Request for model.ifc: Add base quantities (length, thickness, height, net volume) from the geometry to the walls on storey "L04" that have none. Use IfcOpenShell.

First a look at what the model holds.

```python
import ifcopenshell
import ifcopenshell.util.element
import ifcopenshell.util.unit

model = ifcopenshell.open("model.ifc")
print(model.schema)
for unit_type in ("LENGTHUNIT", "AREAUNIT", "VOLUMEUNIT"):
    print(unit_type, ifcopenshell.util.unit.calculate_unit_scale(model, unit_type))
storey = next(s for s in model.by_type("IfcBuildingStorey") if s.Name == "L04")
walls = [e for e in ifcopenshell.util.element.get_decomposition(storey) if e.is_a("IfcWall")]
for e in sorted(walls, key=lambda e: e.id()):
    print(e.id(), e.is_a(), e.Name, list(ifcopenshell.util.element.get_psets(e, qtos_only=True)), sep=" | ")
```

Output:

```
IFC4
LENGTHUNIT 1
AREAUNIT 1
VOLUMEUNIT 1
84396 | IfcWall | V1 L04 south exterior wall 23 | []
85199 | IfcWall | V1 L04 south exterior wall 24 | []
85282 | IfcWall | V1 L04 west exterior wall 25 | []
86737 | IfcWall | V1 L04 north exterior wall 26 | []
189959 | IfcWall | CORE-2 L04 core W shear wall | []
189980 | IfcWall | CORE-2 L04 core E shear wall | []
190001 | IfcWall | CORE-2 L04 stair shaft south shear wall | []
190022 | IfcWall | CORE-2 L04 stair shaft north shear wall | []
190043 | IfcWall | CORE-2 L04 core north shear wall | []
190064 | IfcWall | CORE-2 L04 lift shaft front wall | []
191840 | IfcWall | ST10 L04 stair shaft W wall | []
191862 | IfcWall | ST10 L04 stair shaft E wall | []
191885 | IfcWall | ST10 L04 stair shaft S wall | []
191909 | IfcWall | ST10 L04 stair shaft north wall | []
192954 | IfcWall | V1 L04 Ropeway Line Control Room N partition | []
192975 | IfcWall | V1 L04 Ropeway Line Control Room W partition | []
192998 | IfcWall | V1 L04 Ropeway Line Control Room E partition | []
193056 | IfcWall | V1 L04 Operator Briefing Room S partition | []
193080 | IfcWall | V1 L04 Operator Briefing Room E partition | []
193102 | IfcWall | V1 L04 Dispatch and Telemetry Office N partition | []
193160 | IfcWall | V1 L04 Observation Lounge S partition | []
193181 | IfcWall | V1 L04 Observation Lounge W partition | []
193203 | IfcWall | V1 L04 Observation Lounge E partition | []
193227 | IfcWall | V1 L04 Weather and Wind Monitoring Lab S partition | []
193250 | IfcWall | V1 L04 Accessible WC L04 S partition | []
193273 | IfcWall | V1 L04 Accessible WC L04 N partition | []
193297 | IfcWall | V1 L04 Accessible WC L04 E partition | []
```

```python
import ifcopenshell
import ifcopenshell.api.pset
import ifcopenshell.geom
import ifcopenshell.util.element
import ifcopenshell.util.shape
import ifcopenshell.util.unit

model = ifcopenshell.open("model.ifc")
unit_scale = ifcopenshell.util.unit.calculate_unit_scale(model)
volume_scale = ifcopenshell.util.unit.calculate_unit_scale(model, "VOLUMEUNIT")
settings = ifcopenshell.geom.settings()

storey = next(s for s in model.by_type("IfcBuildingStorey") if s.Name == "L04")
walls = [e for e in ifcopenshell.util.element.get_decomposition(storey) if e.is_a("IfcWall")]

for e in sorted(walls, key=lambda e: e.id()):
    if ifcopenshell.util.element.get_psets(e, qtos_only=True, should_inherit=False):
        continue
    # Geometry comes back in metres, in the element's own axes.
    shape = ifcopenshell.geom.create_shape(settings, e)
    values = {
        "Length": ifcopenshell.util.shape.get_x(shape.geometry) / unit_scale,
        "Width": ifcopenshell.util.shape.get_y(shape.geometry) / unit_scale,
        "Height": ifcopenshell.util.shape.get_z(shape.geometry) / unit_scale,
        "NetVolume": ifcopenshell.util.shape.get_volume(shape.geometry) / volume_scale,
    }
    qto = ifcopenshell.api.pset.add_qto(model, product=e, name="Qto_WallBaseQuantities")
    ifcopenshell.api.pset.edit_qto(model, qto=qto, properties=values)
    print(e.id(), {k: round(v, 3) for k, v in values.items()})

model.write("model_v2.ifc")
```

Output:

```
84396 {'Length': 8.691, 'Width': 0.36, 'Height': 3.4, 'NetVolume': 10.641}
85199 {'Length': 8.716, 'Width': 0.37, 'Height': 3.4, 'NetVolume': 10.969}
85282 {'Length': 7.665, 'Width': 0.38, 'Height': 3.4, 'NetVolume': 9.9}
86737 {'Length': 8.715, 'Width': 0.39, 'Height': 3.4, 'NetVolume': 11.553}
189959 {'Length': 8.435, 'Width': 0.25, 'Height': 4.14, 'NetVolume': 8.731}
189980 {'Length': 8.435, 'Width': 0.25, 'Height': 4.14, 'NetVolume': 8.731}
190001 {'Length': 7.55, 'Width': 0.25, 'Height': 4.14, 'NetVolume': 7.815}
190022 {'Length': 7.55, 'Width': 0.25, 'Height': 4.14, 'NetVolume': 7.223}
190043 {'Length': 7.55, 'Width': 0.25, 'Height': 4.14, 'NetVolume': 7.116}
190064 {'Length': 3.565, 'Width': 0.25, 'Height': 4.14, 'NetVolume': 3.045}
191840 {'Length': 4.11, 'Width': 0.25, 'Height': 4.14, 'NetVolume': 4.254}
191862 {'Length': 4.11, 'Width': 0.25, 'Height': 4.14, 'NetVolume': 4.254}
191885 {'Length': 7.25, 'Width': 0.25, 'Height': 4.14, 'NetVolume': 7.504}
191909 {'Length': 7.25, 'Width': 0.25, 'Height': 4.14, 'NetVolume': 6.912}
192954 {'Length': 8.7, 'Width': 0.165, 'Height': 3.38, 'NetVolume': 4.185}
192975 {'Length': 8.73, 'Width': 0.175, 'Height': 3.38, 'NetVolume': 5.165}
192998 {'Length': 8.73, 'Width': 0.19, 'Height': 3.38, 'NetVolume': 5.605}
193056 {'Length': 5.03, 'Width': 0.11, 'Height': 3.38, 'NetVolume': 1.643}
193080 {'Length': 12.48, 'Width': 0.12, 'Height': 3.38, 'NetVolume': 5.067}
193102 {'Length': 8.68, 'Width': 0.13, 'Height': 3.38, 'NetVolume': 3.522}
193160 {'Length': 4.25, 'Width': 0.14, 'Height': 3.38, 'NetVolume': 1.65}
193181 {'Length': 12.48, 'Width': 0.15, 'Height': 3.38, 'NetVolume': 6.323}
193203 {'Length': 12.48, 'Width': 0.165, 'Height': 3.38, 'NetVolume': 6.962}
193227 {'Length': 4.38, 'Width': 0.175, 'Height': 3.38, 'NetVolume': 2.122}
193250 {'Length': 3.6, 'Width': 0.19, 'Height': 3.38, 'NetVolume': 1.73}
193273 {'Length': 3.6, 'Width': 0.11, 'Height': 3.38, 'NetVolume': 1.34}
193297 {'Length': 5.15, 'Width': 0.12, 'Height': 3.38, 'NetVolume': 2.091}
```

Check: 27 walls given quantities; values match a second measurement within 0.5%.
